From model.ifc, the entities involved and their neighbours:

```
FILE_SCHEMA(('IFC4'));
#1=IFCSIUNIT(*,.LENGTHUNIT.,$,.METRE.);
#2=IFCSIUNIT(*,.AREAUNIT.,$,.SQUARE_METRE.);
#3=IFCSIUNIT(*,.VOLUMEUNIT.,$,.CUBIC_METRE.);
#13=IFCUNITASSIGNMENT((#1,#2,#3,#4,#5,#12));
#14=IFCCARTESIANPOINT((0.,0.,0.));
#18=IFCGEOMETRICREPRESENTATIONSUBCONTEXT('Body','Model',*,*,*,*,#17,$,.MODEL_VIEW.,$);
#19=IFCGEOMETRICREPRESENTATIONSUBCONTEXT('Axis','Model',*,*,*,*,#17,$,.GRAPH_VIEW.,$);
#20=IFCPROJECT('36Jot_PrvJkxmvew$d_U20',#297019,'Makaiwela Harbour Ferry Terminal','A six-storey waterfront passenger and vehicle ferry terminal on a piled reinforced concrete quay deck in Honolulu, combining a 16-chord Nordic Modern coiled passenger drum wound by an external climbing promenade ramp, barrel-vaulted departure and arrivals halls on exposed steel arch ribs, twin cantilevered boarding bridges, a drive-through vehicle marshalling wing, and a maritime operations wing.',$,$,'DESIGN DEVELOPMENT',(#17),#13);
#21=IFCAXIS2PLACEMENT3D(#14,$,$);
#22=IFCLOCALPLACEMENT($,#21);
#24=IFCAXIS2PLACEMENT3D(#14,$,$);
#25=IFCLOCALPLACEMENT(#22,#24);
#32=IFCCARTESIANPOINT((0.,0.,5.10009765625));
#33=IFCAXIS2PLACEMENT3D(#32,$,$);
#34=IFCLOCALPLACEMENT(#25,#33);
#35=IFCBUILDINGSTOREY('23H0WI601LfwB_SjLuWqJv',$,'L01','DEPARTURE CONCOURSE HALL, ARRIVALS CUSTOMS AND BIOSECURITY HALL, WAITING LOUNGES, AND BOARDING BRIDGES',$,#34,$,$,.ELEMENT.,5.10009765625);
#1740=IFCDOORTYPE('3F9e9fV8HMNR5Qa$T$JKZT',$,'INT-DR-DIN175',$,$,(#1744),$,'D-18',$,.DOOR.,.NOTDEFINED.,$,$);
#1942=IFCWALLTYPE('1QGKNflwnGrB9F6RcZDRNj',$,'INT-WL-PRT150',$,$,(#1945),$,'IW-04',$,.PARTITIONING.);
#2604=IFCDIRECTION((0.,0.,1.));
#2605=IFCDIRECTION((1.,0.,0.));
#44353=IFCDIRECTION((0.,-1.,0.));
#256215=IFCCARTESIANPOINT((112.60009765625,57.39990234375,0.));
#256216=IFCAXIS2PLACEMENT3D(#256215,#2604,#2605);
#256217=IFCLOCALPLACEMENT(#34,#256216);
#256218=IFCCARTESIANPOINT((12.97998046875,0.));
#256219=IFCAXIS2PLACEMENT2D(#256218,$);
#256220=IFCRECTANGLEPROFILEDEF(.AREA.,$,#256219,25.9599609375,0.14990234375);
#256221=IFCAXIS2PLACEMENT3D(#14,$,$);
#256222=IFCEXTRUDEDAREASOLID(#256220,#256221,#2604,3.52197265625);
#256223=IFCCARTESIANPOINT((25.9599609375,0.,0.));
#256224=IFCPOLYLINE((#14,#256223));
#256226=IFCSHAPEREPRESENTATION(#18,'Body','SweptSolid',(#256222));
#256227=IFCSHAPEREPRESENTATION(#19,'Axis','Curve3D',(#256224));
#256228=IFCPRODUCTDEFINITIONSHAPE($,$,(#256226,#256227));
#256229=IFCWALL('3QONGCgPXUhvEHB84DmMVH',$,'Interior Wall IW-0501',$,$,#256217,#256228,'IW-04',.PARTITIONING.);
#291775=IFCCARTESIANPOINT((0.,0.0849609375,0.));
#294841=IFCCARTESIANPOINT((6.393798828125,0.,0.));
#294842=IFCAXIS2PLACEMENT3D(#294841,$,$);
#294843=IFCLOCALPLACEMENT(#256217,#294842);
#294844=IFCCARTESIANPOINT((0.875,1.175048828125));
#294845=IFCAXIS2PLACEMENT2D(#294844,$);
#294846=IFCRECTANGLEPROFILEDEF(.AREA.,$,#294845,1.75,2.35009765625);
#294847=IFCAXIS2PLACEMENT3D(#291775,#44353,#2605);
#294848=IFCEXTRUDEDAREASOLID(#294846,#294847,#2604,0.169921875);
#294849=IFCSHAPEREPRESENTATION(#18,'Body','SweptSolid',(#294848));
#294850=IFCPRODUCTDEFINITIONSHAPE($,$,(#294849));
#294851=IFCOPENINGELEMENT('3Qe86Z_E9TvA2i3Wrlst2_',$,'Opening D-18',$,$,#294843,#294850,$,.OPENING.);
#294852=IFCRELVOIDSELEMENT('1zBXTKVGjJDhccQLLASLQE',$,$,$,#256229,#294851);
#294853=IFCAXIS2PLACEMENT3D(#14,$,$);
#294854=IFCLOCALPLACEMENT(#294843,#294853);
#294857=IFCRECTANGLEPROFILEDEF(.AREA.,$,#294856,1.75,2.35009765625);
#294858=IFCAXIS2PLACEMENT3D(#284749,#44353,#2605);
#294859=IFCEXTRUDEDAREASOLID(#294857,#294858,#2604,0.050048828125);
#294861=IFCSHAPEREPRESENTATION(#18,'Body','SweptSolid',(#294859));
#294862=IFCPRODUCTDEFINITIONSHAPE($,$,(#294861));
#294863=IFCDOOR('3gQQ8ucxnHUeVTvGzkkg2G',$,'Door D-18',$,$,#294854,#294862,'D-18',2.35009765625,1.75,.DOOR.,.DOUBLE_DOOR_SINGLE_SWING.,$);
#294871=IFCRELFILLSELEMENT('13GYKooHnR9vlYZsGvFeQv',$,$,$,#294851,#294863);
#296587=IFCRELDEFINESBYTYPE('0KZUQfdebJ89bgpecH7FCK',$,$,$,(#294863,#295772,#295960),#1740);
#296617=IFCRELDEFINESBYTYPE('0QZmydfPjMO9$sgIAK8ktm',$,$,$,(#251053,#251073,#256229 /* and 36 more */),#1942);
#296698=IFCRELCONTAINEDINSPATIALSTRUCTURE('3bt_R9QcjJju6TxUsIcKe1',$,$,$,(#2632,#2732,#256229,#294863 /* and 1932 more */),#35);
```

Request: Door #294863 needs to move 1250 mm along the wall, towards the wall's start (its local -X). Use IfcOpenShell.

```python
import ifcopenshell
import ifcopenshell.api.geometry
import ifcopenshell.util.placement

model = ifcopenshell.open("model.ifc")

door = model.by_id(294863)
opening = door.FillsVoids[0].RelatingOpeningElement
wall = opening.VoidsElements[0].RelatingBuildingElement

wall_matrix = ifcopenshell.util.placement.get_local_placement(wall.ObjectPlacement)
shift = wall_matrix[:3, 0] * -1.25
before = ifcopenshell.util.placement.get_local_placement(door.ObjectPlacement)[:3, 3].copy()

# The door is placed relative to its opening, so it follows when the opening moves.
matrix = ifcopenshell.util.placement.get_local_placement(opening.ObjectPlacement)
matrix[:3, 3] += shift
ifcopenshell.api.geometry.edit_object_placement(
    model, product=opening, matrix=matrix, is_si=False, should_transform_children=True
)

after = ifcopenshell.util.placement.get_local_placement(door.ObjectPlacement)[:3, 3]
print("door moved by", (after - before).round(3) + 0.0)

model.write("model_v2.ifc")
```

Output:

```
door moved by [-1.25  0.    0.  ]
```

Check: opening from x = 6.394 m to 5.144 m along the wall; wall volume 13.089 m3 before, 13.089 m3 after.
